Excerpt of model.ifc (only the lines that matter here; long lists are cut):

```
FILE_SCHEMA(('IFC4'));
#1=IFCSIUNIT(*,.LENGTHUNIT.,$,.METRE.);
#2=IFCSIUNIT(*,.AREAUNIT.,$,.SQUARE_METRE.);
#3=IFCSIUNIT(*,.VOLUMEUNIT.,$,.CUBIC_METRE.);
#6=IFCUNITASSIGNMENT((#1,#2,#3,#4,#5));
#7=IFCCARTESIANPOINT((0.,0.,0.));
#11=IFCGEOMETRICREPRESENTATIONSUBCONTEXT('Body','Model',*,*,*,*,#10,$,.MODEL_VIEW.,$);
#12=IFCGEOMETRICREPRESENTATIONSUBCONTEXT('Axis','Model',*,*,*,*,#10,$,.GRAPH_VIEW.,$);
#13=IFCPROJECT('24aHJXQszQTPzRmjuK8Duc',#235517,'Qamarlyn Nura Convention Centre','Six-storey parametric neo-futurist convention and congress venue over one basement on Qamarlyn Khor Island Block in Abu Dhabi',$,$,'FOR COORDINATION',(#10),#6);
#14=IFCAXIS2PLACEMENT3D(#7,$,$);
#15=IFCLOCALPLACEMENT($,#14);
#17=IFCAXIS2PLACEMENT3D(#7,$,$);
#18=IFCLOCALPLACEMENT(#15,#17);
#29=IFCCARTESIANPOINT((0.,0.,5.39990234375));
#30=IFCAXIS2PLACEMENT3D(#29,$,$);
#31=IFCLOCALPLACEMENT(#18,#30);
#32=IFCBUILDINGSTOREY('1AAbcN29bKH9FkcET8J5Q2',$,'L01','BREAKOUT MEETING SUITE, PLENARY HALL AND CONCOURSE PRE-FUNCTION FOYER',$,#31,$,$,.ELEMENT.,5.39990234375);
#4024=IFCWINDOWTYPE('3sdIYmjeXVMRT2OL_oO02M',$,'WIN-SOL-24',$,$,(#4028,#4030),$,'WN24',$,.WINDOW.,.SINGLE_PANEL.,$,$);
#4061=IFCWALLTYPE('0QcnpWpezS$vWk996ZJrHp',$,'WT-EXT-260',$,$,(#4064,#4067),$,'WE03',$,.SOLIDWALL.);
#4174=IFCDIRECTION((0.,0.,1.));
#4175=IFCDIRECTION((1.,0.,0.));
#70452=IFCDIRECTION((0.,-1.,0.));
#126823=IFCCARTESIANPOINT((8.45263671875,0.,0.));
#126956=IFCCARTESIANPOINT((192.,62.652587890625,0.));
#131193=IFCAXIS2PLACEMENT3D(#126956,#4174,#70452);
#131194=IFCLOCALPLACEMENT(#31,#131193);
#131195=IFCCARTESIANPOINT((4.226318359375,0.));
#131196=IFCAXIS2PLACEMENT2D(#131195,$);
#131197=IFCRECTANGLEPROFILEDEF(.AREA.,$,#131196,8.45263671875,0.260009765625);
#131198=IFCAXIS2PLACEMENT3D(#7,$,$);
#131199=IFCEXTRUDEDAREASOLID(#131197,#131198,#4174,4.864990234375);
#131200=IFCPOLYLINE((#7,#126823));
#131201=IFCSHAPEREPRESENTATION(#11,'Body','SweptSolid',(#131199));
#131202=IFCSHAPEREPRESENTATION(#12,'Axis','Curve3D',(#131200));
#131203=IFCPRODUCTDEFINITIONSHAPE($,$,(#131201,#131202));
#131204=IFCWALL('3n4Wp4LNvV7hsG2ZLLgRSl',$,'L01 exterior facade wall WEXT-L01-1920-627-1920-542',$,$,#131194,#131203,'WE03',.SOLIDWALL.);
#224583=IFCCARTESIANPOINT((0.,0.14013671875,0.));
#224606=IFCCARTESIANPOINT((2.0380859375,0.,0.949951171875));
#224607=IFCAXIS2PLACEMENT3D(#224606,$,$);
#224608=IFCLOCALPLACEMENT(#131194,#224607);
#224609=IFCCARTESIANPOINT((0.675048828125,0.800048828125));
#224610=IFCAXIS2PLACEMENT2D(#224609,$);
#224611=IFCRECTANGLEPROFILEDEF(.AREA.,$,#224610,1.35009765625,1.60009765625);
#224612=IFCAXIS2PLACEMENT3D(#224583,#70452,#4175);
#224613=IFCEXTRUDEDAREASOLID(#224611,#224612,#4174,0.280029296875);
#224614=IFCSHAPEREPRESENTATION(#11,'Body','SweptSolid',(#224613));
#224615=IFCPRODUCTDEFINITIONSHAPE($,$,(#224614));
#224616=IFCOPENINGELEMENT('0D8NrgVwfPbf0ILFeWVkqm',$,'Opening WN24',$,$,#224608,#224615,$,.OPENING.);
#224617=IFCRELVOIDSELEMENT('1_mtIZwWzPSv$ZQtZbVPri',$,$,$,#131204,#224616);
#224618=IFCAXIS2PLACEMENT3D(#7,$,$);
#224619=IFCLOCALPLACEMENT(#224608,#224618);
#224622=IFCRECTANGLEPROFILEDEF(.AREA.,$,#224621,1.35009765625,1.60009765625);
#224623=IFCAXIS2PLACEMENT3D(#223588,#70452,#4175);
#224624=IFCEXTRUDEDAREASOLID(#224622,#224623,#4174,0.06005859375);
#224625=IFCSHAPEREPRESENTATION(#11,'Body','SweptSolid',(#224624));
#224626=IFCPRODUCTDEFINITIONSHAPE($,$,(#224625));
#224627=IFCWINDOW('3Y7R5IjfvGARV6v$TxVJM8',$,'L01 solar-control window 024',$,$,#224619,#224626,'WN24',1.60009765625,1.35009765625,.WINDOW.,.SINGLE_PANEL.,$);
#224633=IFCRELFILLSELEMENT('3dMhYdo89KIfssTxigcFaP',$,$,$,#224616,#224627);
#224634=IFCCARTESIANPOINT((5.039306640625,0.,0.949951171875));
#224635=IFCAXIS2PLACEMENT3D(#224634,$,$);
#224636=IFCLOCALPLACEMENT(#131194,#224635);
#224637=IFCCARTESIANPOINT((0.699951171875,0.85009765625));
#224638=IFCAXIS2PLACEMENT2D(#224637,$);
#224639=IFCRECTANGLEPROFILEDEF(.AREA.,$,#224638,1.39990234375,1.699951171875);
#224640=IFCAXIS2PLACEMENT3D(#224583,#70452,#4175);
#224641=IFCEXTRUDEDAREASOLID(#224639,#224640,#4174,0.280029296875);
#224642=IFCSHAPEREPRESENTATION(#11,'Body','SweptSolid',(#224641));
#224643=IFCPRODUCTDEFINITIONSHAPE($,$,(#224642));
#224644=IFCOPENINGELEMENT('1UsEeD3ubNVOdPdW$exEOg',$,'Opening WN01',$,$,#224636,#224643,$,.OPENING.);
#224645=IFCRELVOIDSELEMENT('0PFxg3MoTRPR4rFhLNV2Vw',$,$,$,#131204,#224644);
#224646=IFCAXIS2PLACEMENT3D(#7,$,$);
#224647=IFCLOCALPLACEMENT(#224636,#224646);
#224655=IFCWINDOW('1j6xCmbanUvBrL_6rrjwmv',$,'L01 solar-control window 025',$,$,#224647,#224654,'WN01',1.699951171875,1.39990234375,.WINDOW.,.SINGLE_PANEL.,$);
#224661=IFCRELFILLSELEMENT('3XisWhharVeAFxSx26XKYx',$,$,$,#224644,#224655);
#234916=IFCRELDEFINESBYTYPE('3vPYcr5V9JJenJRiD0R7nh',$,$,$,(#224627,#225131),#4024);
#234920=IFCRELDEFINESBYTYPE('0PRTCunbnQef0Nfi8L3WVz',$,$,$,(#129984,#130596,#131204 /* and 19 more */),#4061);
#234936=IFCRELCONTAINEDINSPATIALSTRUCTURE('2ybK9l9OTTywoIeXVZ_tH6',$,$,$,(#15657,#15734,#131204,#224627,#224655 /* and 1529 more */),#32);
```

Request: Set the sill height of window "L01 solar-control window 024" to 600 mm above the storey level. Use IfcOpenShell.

```python
import numpy as np
import ifcopenshell
import ifcopenshell.api.geometry
import ifcopenshell.geom
import ifcopenshell.util.element
import ifcopenshell.util.placement
import ifcopenshell.util.shape
import ifcopenshell.util.unit

model = ifcopenshell.open("model.ifc")
unit_scale = ifcopenshell.util.unit.calculate_unit_scale(model)

window = model.by_guid("3Y7R5IjfvGARV6v$TxVJM8")
opening = window.FillsVoids[0].RelatingOpeningElement
storey = ifcopenshell.util.element.get_container(window, ifc_class="IfcBuildingStorey")
level = ifcopenshell.util.placement.get_local_placement(storey.ObjectPlacement)[2, 3]

# The opening's origin need not be at the sill, so measure its lowest point.
shape = ifcopenshell.geom.create_shape(ifcopenshell.geom.settings(), opening)
bottom = ifcopenshell.util.shape.get_shape_bottom_elevation(shape, shape.geometry) / unit_scale
dz = level + 0.6 - bottom

shift = np.array([0.0, 0.0, dz])
# The window is placed relative to its opening, so it follows when the opening moves.
matrix = ifcopenshell.util.placement.get_local_placement(opening.ObjectPlacement)
matrix[:3, 3] += shift
ifcopenshell.api.geometry.edit_object_placement(
    model, product=opening, matrix=matrix, is_si=False, should_transform_children=True
)

print(f"moved by {dz * unit_scale:+.3f} m")

model.write("model-out.ifc")
```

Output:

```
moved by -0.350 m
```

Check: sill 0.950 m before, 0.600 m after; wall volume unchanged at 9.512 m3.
